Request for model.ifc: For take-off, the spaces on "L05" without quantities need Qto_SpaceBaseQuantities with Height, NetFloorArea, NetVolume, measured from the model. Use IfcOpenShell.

First a look at what the model holds.

```python
import ifcopenshell
import ifcopenshell.util.element
import ifcopenshell.util.unit

model = ifcopenshell.open("model.ifc")
print(model.schema)
for unit_type in ("LENGTHUNIT", "AREAUNIT", "VOLUMEUNIT"):
    print(unit_type, ifcopenshell.util.unit.calculate_unit_scale(model, unit_type))
storey = next(s for s in model.by_type("IfcBuildingStorey") if s.Name == "L05")
spaces = [e for e in ifcopenshell.util.element.get_decomposition(storey) if e.is_a("IfcSpace")]
for e in sorted(spaces, key=lambda e: e.id()):
    print(e.id(), e.is_a(), e.Name, list(ifcopenshell.util.element.get_psets(e, qtos_only=True)), sep=" | ")
```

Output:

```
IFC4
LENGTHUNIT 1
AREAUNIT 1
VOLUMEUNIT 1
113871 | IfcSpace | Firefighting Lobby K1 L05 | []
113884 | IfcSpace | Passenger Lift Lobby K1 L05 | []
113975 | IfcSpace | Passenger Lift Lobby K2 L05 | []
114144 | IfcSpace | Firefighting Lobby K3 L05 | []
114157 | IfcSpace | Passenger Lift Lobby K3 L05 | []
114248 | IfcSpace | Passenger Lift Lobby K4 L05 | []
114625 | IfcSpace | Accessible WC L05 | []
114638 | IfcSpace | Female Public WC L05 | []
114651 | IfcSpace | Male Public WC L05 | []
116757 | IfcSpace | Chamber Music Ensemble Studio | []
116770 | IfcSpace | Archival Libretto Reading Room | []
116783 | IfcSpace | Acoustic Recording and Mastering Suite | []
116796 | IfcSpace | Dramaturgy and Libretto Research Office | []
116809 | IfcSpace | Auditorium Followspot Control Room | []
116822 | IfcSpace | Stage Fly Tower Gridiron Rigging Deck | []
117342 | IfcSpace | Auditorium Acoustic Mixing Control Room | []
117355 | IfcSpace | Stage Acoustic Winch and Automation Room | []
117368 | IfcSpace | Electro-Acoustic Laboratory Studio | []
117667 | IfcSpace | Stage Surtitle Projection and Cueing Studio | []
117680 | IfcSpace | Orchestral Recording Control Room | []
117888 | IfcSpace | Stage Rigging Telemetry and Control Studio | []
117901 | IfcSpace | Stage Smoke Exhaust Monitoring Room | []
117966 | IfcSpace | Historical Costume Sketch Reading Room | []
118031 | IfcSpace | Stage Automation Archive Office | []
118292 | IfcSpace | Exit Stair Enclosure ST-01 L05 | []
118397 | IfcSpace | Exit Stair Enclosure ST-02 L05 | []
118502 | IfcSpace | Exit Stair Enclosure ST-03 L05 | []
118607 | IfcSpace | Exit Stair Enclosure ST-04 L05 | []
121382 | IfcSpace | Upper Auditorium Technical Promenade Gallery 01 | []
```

```python
import ifcopenshell
import ifcopenshell.api.pset
import ifcopenshell.geom
import ifcopenshell.util.element
import ifcopenshell.util.shape
import ifcopenshell.util.unit

model = ifcopenshell.open("model.ifc")
unit_scale = ifcopenshell.util.unit.calculate_unit_scale(model)
area_scale = ifcopenshell.util.unit.calculate_unit_scale(model, "AREAUNIT")
volume_scale = ifcopenshell.util.unit.calculate_unit_scale(model, "VOLUMEUNIT")
settings = ifcopenshell.geom.settings()

storey = next(s for s in model.by_type("IfcBuildingStorey") if s.Name == "L05")
spaces = [e for e in ifcopenshell.util.element.get_decomposition(storey) if e.is_a("IfcSpace")]

for e in sorted(spaces, key=lambda e: e.id()):
    if ifcopenshell.util.element.get_psets(e, qtos_only=True, should_inherit=False):
        continue
    # Geometry comes back in metres, in the element's own axes.
    shape = ifcopenshell.geom.create_shape(settings, e)
    values = {
        "Height": ifcopenshell.util.shape.get_z(shape.geometry) / unit_scale,
        "NetFloorArea": ifcopenshell.util.shape.get_footprint_area(shape.geometry) / area_scale,
        "NetVolume": ifcopenshell.util.shape.get_volume(shape.geometry) / volume_scale,
    }
    qto = ifcopenshell.api.pset.add_qto(model, product=e, name="Qto_SpaceBaseQuantities")
    ifcopenshell.api.pset.edit_qto(model, qto=qto, properties=values)
    print(e.id(), {k: round(v, 3) for k, v in values.items()})

model.write("model_rev.ifc")
```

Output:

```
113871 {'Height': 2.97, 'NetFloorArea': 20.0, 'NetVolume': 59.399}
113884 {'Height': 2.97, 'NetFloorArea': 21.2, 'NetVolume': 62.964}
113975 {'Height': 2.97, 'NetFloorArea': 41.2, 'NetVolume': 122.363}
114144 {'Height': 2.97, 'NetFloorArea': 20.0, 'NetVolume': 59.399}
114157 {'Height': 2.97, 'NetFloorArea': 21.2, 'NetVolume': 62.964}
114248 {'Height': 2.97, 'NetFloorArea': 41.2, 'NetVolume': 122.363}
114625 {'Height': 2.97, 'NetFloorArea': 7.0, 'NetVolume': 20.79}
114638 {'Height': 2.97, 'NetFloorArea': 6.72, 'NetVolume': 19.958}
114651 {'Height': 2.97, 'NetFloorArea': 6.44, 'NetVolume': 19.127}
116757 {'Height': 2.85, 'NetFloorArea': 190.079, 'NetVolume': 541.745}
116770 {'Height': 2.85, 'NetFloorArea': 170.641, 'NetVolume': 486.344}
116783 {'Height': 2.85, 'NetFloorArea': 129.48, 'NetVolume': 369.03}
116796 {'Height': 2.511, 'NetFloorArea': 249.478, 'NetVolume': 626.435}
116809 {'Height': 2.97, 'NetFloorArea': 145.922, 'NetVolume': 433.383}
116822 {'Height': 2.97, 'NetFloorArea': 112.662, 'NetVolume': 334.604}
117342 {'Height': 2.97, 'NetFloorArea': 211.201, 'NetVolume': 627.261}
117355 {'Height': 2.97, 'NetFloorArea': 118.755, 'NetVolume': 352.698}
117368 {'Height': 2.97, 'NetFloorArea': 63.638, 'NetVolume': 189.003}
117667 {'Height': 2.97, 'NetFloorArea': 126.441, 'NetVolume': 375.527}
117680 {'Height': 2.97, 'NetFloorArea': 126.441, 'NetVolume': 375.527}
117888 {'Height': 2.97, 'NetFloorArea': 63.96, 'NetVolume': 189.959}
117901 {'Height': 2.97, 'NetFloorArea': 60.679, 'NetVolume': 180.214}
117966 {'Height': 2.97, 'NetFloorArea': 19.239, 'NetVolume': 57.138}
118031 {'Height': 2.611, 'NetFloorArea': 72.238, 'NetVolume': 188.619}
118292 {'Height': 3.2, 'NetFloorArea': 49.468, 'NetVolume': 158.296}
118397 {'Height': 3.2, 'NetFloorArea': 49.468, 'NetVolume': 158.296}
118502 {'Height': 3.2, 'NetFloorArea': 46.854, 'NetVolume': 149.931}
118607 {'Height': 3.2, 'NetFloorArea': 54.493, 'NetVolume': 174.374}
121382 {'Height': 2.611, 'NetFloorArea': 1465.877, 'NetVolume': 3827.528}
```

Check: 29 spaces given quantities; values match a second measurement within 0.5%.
